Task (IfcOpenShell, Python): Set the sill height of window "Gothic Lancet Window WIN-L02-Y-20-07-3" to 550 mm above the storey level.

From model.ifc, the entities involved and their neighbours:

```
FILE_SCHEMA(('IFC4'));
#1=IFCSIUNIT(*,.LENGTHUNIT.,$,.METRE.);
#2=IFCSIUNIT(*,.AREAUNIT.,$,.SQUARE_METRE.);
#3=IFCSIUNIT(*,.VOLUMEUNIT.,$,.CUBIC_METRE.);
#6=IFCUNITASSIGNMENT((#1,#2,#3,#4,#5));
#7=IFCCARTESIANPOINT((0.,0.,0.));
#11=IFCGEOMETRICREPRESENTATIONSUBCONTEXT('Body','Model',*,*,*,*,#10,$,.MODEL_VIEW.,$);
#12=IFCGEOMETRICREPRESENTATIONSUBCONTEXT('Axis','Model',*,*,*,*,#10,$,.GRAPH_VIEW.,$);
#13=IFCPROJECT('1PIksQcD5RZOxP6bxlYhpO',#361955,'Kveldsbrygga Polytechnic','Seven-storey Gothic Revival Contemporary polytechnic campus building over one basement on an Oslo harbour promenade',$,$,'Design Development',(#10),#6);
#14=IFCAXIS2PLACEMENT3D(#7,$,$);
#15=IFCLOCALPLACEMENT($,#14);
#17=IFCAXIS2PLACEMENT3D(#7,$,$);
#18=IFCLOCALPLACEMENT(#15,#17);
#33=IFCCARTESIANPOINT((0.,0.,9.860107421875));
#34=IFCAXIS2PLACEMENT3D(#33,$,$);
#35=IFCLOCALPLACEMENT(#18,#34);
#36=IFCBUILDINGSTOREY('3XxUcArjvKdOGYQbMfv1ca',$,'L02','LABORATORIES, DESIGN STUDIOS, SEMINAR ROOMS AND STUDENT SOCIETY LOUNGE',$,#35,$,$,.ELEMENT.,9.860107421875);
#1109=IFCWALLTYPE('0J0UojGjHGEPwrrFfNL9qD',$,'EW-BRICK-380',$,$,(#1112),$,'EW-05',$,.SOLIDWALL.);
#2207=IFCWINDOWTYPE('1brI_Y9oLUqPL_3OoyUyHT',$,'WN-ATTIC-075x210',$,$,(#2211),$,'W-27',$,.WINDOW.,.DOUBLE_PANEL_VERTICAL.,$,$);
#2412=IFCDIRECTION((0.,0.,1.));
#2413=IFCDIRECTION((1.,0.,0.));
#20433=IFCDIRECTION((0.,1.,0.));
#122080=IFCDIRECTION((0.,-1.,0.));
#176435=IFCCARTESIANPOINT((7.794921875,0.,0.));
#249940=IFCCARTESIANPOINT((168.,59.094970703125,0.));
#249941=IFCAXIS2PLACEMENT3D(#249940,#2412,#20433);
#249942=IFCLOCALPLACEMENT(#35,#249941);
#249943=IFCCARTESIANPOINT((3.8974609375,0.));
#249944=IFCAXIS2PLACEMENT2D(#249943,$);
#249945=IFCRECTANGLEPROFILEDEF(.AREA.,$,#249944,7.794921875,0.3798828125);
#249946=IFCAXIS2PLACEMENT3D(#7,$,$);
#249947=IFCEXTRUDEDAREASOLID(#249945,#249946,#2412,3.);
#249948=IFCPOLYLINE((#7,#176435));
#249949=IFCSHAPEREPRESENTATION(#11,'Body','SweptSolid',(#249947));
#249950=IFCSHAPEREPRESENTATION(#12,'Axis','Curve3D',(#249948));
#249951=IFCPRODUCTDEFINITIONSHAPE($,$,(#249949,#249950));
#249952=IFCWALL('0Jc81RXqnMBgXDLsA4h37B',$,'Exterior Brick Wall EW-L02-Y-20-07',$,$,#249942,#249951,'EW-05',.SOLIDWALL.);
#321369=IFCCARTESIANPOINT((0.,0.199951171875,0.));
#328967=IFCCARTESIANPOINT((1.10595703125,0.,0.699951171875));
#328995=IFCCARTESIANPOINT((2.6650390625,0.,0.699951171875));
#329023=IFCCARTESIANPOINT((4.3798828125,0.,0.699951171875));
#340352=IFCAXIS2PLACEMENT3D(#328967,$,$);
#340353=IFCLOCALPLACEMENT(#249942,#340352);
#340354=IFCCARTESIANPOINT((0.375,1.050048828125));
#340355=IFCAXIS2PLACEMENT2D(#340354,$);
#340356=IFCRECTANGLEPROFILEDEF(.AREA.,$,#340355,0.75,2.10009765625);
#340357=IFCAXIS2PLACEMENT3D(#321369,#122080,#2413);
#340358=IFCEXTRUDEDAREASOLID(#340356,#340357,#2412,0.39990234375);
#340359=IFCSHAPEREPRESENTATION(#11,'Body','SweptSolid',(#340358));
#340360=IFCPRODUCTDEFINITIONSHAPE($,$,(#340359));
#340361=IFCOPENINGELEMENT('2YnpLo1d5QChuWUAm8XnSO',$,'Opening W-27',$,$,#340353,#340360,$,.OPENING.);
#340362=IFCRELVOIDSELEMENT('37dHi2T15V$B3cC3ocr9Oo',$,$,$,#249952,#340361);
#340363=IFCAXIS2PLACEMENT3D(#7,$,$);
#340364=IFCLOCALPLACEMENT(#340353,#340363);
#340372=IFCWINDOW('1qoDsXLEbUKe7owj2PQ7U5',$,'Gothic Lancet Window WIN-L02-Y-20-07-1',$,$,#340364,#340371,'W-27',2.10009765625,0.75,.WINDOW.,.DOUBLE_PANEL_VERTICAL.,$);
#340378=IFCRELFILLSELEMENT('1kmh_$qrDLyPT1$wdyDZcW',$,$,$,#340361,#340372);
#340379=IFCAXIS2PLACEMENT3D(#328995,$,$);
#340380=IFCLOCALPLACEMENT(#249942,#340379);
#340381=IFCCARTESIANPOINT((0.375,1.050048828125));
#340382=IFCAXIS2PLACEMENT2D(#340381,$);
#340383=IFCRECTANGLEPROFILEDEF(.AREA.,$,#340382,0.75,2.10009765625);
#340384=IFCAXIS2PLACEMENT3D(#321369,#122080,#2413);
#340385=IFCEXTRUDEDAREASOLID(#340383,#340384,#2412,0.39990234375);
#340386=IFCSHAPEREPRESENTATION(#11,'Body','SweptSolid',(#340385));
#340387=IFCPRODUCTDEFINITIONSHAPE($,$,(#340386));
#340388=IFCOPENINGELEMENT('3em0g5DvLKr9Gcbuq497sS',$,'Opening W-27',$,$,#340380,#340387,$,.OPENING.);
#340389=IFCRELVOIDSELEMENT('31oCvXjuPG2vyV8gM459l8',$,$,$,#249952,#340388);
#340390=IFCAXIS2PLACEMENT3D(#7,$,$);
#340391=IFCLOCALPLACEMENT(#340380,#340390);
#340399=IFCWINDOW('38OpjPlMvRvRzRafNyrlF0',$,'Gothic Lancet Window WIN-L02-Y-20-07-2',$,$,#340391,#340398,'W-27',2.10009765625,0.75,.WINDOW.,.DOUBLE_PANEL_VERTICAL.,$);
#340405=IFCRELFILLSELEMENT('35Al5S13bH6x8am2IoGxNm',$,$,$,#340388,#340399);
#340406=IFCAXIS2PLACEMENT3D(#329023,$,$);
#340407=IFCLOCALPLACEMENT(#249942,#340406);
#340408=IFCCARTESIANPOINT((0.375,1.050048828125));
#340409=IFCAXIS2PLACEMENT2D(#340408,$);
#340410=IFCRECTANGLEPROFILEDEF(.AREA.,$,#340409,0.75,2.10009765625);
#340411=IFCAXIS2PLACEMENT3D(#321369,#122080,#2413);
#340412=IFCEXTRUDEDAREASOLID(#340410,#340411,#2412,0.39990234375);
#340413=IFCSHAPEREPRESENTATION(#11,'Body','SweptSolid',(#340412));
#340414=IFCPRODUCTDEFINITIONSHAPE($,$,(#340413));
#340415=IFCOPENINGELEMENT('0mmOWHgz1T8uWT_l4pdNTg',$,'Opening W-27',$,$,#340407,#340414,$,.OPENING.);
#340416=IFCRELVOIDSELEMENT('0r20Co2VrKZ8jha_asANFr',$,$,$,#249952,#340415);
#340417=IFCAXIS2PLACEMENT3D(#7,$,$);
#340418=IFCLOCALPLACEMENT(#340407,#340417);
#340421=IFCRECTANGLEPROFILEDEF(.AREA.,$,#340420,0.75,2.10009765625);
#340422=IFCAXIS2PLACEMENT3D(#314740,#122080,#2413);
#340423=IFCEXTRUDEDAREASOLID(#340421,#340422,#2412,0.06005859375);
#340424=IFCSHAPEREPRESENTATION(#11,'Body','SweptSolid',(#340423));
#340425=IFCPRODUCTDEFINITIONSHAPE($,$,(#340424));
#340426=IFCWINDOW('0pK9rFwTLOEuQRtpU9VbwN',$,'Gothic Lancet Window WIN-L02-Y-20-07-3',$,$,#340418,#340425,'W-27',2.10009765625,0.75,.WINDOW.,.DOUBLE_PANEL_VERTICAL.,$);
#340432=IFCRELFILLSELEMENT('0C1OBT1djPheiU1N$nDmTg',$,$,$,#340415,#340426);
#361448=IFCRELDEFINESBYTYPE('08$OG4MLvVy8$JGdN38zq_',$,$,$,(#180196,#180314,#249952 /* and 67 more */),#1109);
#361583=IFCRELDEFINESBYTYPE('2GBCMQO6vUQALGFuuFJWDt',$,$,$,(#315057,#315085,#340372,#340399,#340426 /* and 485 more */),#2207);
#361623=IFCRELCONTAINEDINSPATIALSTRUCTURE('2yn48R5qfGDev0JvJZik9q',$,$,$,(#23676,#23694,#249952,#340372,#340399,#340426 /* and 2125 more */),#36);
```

```python
import numpy as np
import ifcopenshell
import ifcopenshell.api.geometry
import ifcopenshell.geom
import ifcopenshell.util.element
import ifcopenshell.util.placement
import ifcopenshell.util.shape
import ifcopenshell.util.unit

model = ifcopenshell.open("model.ifc")
unit_scale = ifcopenshell.util.unit.calculate_unit_scale(model)

window = model.by_id(340426)
opening = window.FillsVoids[0].RelatingOpeningElement
storey = ifcopenshell.util.element.get_container(window, ifc_class="IfcBuildingStorey")
level = ifcopenshell.util.placement.get_local_placement(storey.ObjectPlacement)[2, 3]

# The opening's origin need not be at the sill, so measure its lowest point.
shape = ifcopenshell.geom.create_shape(ifcopenshell.geom.settings(), opening)
bottom = ifcopenshell.util.shape.get_shape_bottom_elevation(shape, shape.geometry) / unit_scale
dz = level + 0.55 - bottom

shift = np.array([0.0, 0.0, dz])
# The window is placed relative to its opening, so it follows when the opening moves.
matrix = ifcopenshell.util.placement.get_local_placement(opening.ObjectPlacement)
matrix[:3, 3] += shift
ifcopenshell.api.geometry.edit_object_placement(
    model, product=opening, matrix=matrix, is_si=False, should_transform_children=True
)

print(f"moved by {dz * unit_scale:+.3f} m")

model.write("model_rev.ifc")
```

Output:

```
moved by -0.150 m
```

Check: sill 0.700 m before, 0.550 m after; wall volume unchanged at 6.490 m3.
